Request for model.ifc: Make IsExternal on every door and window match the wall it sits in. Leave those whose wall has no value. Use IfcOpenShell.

First a look at what the model holds.

```python
import ifcopenshell
import ifcopenshell.util.element

model = ifcopenshell.open("model.ifc")
print(model.schema)
seen = {}
for e in model.by_type("IfcDoor") + model.by_type("IfcWindow"):
    if not e.FillsVoids:
        continue
    host = e.FillsVoids[0].RelatingOpeningElement.VoidsElements[0].RelatingBuildingElement
    own = ifcopenshell.util.element.get_pset(e, f"Pset_{e.is_a()[3:].removesuffix('StandardCase')}Common", "IsExternal")
    wall = ifcopenshell.util.element.get_pset(host, "Pset_WallCommon", "IsExternal")
    seen[e.is_a(), own, wall] = seen.get((e.is_a(), own, wall), 0) + 1
for (cls, own, wall), count in sorted(seen.items(), key=str):
    print(count, cls, "IsExternal:", own, "| host wall:", wall)
```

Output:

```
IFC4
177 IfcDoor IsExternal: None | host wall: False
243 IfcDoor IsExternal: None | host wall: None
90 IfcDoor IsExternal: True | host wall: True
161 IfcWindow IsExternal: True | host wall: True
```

```python
import ifcopenshell
import ifcopenshell.api.pset
import ifcopenshell.util.element

model = ifcopenshell.open("model.ifc")

count = 0
for ifc_class, pset_name in (("IfcDoor", "Pset_DoorCommon"), ("IfcWindow", "Pset_WindowCommon")):
    for e in model.by_type(ifc_class):
        if not e.FillsVoids:
            continue
        host = e.FillsVoids[0].RelatingOpeningElement.VoidsElements[0].RelatingBuildingElement
        external = ifcopenshell.util.element.get_pset(host, "Pset_WallCommon", "IsExternal")
        if external is None or ifcopenshell.util.element.get_pset(e, pset_name, "IsExternal") == external:
            continue
        pset = ifcopenshell.api.pset.add_pset(model, product=e, name=pset_name)
        ifcopenshell.api.pset.edit_pset(model, pset=pset, properties={"IsExternal": external})
        count += 1

print(count, "updated")

model.write("model-out.ifc")
```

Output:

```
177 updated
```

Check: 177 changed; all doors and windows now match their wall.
